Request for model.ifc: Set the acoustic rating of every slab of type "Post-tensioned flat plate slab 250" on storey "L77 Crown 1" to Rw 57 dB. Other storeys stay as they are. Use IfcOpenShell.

First a look at what the model holds.

```python
import ifcopenshell
import ifcopenshell.util.element

model = ifcopenshell.open("model.ifc")
print(model.schema)
storey = next(s for s in model.by_type("IfcBuildingStorey") if s.Name == "L77 Crown 1")
slabs = [e for e in ifcopenshell.util.element.get_decomposition(storey) if e.is_a("IfcSlab")]
seen = {}
for e in slabs:
    element_type = ifcopenshell.util.element.get_type(e)
    key = (element_type.Name if element_type != e and element_type else None, ifcopenshell.util.element.get_pset(e, "Pset_SlabCommon", "AcousticRating"))
    seen[key] = seen.get(key, 0) + 1
for (name, value), count in sorted(seen.items(), key=str):
    print(count, "x", name, "|", value)
```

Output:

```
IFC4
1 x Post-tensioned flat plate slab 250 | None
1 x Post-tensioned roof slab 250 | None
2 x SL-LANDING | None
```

```python
import ifcopenshell
import ifcopenshell.api.pset
import ifcopenshell.util.element

model = ifcopenshell.open("model.ifc")

storey = next(s for s in model.by_type("IfcBuildingStorey") if s.Name == "L77 Crown 1")
slabs = [e for e in ifcopenshell.util.element.get_decomposition(storey) if e.is_a("IfcSlab")]

count = 0
for e in slabs:
    element_type = ifcopenshell.util.element.get_type(e)
    if element_type in (None, e) or element_type.Name != "Post-tensioned flat plate slab 250":
        continue
    found = ifcopenshell.util.element.get_pset(e, "Pset_SlabCommon", should_inherit=False)
    if found:
        pset = model.by_id(found["id"])
        if len(ifcopenshell.util.element.get_elements_by_pset(pset)) > 1:
            pset = ifcopenshell.api.pset.unshare_pset(model, products=[e], pset=pset)[0]
    else:
        pset = ifcopenshell.api.pset.add_pset(model, product=e, name="Pset_SlabCommon")
    ifcopenshell.api.pset.edit_pset(model, pset=pset, properties={"AcousticRating": "Rw 57 dB"})
    count += 1

print(count, "slabs updated")

model.write("model_edited.ifc")
```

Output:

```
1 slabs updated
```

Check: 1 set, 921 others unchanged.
